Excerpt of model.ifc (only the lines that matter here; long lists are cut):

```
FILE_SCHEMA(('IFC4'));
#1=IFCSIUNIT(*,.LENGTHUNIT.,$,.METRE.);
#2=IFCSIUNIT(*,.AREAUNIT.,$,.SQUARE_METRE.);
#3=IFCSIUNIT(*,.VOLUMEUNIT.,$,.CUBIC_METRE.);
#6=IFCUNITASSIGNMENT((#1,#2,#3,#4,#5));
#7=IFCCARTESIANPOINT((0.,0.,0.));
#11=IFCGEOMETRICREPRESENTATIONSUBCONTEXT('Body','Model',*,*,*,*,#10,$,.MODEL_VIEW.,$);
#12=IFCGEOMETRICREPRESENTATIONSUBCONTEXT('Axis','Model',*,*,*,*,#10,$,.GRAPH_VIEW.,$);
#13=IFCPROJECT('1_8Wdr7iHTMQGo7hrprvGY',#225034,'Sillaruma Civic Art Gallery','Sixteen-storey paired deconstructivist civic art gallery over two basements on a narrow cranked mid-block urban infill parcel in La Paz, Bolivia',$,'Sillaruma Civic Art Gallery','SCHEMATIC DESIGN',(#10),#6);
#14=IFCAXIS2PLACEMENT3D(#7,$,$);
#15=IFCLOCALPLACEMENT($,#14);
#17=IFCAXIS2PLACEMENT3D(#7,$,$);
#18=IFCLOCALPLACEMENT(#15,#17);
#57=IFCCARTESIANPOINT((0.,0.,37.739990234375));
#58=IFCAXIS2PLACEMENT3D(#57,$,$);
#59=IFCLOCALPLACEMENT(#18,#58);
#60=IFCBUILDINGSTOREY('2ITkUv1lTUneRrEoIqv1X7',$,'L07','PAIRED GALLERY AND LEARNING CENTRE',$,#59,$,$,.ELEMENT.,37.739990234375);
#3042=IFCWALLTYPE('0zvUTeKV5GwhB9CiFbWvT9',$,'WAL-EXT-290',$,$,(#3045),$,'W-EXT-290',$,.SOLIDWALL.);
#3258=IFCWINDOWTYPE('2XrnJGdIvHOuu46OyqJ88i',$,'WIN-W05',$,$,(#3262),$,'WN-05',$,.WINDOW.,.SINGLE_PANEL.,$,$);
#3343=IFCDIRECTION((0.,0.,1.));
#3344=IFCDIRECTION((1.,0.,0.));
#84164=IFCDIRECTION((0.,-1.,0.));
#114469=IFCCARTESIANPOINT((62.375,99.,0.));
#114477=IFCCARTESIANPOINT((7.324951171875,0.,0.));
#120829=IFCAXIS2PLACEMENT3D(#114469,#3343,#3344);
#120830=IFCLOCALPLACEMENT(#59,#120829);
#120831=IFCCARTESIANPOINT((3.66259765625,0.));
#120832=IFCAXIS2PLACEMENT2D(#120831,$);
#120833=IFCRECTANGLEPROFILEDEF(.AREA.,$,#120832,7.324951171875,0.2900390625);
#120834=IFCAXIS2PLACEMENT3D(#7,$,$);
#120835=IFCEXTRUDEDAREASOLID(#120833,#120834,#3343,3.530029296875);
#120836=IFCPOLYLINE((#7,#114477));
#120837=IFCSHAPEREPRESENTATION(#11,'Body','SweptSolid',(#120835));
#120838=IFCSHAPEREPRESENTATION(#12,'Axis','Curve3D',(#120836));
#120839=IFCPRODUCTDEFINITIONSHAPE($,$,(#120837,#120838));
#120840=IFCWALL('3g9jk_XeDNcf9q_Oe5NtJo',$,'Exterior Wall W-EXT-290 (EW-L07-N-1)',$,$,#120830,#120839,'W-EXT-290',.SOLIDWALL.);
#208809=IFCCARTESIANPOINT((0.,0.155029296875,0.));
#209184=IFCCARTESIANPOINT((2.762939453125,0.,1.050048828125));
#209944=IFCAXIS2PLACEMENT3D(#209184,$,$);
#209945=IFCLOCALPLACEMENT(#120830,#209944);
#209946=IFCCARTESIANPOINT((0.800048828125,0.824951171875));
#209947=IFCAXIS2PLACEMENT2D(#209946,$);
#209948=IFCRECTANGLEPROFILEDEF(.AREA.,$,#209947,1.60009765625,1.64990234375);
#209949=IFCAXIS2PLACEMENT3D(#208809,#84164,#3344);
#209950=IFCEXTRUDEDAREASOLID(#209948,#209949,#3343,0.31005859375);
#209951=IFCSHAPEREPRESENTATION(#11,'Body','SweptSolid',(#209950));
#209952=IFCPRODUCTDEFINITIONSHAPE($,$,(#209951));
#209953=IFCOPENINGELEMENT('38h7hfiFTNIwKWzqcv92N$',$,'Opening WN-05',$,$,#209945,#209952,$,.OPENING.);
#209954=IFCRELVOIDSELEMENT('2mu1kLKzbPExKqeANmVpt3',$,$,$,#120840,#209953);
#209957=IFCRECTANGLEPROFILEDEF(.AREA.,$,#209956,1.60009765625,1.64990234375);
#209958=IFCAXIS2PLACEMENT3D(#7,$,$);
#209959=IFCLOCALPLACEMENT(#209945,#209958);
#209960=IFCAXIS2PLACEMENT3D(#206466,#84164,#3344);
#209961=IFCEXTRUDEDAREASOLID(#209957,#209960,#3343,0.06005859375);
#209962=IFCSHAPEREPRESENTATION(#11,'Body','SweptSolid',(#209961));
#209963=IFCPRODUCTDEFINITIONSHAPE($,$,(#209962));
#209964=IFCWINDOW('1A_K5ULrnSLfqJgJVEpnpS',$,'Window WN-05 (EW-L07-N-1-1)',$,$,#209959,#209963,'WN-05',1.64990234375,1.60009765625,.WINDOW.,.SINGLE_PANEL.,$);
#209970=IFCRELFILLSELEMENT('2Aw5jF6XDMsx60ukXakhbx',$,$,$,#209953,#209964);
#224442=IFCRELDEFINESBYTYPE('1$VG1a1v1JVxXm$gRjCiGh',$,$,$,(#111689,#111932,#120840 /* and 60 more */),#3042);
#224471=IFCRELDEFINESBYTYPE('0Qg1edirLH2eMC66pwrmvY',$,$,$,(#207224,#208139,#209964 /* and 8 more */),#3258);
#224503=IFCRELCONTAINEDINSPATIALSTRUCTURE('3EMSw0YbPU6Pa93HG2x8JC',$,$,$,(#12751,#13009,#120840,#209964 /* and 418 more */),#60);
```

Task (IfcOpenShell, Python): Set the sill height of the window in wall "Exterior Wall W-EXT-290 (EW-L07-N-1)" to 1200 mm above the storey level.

```python
import numpy as np
import ifcopenshell
import ifcopenshell.api.geometry
import ifcopenshell.geom
import ifcopenshell.util.element
import ifcopenshell.util.placement
import ifcopenshell.util.shape
import ifcopenshell.util.unit

model = ifcopenshell.open("model.ifc")
unit_scale = ifcopenshell.util.unit.calculate_unit_scale(model)

window = model.by_guid("1A_K5ULrnSLfqJgJVEpnpS")
opening = window.FillsVoids[0].RelatingOpeningElement
storey = ifcopenshell.util.element.get_container(window, ifc_class="IfcBuildingStorey")
level = ifcopenshell.util.placement.get_local_placement(storey.ObjectPlacement)[2, 3]

# The opening's origin need not be at the sill, so measure its lowest point.
shape = ifcopenshell.geom.create_shape(ifcopenshell.geom.settings(), opening)
bottom = ifcopenshell.util.shape.get_shape_bottom_elevation(shape, shape.geometry) / unit_scale
dz = level + 1.2 - bottom

shift = np.array([0.0, 0.0, dz])
# The window is placed relative to its opening, so it follows when the opening moves.
matrix = ifcopenshell.util.placement.get_local_placement(opening.ObjectPlacement)
matrix[:3, 3] += shift
ifcopenshell.api.geometry.edit_object_placement(
    model, product=opening, matrix=matrix, is_si=False, should_transform_children=True
)

print(f"moved by {dz * unit_scale:+.3f} m")

model.write("model_v2.ifc")
```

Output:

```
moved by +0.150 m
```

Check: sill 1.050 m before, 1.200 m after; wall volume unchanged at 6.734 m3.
